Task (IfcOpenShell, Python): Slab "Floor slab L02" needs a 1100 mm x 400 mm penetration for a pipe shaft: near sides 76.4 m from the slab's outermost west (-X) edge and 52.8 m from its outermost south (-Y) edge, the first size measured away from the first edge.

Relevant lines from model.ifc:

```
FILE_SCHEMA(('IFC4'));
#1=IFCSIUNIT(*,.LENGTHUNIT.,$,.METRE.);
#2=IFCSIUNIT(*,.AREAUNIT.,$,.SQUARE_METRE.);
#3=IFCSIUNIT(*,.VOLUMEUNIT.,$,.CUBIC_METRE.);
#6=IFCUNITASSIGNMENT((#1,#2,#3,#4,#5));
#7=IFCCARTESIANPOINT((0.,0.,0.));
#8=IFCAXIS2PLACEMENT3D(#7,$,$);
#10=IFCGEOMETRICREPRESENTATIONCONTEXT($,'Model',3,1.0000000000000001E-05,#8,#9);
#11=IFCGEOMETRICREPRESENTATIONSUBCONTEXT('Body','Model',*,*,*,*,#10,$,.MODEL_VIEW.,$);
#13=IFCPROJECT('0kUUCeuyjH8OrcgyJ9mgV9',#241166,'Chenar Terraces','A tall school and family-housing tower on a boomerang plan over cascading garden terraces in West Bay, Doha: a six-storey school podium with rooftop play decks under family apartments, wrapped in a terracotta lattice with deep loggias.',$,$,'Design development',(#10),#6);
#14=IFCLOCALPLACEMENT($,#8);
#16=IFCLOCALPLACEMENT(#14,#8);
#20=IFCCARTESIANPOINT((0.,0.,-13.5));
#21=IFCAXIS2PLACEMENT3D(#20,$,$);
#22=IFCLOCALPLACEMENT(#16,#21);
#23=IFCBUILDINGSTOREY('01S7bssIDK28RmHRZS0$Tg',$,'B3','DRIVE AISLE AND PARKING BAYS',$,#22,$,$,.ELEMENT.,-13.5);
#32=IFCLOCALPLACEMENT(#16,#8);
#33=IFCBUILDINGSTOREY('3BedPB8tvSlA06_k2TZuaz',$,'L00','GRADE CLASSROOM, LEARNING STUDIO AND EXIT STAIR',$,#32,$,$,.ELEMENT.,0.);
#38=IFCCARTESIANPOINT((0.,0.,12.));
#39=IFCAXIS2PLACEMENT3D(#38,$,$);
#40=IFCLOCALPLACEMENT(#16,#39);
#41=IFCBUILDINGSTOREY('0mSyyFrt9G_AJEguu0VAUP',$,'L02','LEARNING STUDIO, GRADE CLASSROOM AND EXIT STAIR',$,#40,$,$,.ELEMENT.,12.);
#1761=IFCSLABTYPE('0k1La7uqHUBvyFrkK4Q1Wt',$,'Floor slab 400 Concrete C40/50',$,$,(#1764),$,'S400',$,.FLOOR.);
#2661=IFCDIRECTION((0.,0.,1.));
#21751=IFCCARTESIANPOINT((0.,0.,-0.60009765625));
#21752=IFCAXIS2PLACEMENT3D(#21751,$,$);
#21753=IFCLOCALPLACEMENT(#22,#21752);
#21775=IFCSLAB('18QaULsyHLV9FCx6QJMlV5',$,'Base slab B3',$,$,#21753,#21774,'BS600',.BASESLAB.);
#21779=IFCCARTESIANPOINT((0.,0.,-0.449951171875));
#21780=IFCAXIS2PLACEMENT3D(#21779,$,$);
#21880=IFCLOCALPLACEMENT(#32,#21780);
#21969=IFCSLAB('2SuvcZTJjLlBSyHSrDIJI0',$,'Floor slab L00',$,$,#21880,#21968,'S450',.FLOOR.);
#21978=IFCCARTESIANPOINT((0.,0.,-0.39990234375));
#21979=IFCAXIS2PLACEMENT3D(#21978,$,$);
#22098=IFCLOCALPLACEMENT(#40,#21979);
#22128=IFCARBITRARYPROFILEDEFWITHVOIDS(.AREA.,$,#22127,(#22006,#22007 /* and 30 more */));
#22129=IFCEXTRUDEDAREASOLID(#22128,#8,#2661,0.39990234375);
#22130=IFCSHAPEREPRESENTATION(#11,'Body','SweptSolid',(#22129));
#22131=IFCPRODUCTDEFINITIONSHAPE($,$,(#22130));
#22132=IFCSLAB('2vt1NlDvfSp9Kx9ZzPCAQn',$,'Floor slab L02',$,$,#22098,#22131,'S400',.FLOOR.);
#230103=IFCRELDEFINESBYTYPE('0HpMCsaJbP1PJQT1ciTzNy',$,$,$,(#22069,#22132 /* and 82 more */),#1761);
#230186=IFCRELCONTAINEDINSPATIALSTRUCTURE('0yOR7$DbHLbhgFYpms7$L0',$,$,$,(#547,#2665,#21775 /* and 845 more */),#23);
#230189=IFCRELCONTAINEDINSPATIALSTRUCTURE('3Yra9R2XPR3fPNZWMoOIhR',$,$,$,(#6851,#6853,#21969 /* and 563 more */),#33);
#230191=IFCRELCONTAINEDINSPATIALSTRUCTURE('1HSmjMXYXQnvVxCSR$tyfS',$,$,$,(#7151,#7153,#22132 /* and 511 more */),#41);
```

```python
import numpy as np
import ifcopenshell
import ifcopenshell.api.feature
import ifcopenshell.api.geometry
import ifcopenshell.api.root
import ifcopenshell.geom
import ifcopenshell.util.placement
import ifcopenshell.util.representation
import ifcopenshell.util.shape
import ifcopenshell.util.unit

model = ifcopenshell.open("model.ifc")
unit_scale = ifcopenshell.util.unit.calculate_unit_scale(model)
settings = ifcopenshell.geom.settings()


def volume(element):
    """Net volume in cubic metres, openings subtracted."""
    shape = ifcopenshell.geom.create_shape(settings, element)
    return ifcopenshell.util.shape.get_volume(shape.geometry)


slab = model.by_id(22132)
before = volume(slab)

# Extent in the slab's own axes, in metres. The edges named are its -X and -Y sides.
slab_shape = ifcopenshell.geom.create_shape(settings, slab)
vertices = ifcopenshell.util.shape.get_vertices(slab_shape.geometry)
x_min, y_min, bottom = vertices.min(axis=0)
top = vertices[:, 2].max()

opening = ifcopenshell.api.root.create_entity(model, ifc_class="IfcOpeningElement", name="Pipe shaft opening", predefined_type="OPENING")
context = ifcopenshell.util.representation.get_context(model, "Model", "Body", "MODEL_VIEW")
width, depth = 1.1, 0.4
outline = [(0.0, 0.0), (width, 0.0), (width, depth), (0.0, depth), (0.0, 0.0)]
# Overshoot both faces by 50 mm so the cut is clean.
shape = ifcopenshell.api.geometry.add_slab_representation(
    model, context=context, depth=top - bottom + 0.1, polyline=outline
)
ifcopenshell.api.geometry.assign_representation(model, product=opening, representation=shape)

matrix = ifcopenshell.util.placement.get_local_placement(slab.ObjectPlacement)
matrix[:, 3] = matrix @ np.append(np.array([x_min + 76.4, y_min + 52.8, bottom - 0.05]) / unit_scale, 1.0)
ifcopenshell.api.geometry.edit_object_placement(model, product=opening, matrix=matrix, is_si=False)
ifcopenshell.api.feature.add_feature(model, feature=opening, element=slab)

after = volume(slab)

print(f"slab volume {before:.3f} -> {after:.3f} m3")

model.write("model_updated.ifc")
```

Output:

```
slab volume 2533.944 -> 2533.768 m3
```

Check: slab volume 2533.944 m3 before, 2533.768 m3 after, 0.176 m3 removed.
